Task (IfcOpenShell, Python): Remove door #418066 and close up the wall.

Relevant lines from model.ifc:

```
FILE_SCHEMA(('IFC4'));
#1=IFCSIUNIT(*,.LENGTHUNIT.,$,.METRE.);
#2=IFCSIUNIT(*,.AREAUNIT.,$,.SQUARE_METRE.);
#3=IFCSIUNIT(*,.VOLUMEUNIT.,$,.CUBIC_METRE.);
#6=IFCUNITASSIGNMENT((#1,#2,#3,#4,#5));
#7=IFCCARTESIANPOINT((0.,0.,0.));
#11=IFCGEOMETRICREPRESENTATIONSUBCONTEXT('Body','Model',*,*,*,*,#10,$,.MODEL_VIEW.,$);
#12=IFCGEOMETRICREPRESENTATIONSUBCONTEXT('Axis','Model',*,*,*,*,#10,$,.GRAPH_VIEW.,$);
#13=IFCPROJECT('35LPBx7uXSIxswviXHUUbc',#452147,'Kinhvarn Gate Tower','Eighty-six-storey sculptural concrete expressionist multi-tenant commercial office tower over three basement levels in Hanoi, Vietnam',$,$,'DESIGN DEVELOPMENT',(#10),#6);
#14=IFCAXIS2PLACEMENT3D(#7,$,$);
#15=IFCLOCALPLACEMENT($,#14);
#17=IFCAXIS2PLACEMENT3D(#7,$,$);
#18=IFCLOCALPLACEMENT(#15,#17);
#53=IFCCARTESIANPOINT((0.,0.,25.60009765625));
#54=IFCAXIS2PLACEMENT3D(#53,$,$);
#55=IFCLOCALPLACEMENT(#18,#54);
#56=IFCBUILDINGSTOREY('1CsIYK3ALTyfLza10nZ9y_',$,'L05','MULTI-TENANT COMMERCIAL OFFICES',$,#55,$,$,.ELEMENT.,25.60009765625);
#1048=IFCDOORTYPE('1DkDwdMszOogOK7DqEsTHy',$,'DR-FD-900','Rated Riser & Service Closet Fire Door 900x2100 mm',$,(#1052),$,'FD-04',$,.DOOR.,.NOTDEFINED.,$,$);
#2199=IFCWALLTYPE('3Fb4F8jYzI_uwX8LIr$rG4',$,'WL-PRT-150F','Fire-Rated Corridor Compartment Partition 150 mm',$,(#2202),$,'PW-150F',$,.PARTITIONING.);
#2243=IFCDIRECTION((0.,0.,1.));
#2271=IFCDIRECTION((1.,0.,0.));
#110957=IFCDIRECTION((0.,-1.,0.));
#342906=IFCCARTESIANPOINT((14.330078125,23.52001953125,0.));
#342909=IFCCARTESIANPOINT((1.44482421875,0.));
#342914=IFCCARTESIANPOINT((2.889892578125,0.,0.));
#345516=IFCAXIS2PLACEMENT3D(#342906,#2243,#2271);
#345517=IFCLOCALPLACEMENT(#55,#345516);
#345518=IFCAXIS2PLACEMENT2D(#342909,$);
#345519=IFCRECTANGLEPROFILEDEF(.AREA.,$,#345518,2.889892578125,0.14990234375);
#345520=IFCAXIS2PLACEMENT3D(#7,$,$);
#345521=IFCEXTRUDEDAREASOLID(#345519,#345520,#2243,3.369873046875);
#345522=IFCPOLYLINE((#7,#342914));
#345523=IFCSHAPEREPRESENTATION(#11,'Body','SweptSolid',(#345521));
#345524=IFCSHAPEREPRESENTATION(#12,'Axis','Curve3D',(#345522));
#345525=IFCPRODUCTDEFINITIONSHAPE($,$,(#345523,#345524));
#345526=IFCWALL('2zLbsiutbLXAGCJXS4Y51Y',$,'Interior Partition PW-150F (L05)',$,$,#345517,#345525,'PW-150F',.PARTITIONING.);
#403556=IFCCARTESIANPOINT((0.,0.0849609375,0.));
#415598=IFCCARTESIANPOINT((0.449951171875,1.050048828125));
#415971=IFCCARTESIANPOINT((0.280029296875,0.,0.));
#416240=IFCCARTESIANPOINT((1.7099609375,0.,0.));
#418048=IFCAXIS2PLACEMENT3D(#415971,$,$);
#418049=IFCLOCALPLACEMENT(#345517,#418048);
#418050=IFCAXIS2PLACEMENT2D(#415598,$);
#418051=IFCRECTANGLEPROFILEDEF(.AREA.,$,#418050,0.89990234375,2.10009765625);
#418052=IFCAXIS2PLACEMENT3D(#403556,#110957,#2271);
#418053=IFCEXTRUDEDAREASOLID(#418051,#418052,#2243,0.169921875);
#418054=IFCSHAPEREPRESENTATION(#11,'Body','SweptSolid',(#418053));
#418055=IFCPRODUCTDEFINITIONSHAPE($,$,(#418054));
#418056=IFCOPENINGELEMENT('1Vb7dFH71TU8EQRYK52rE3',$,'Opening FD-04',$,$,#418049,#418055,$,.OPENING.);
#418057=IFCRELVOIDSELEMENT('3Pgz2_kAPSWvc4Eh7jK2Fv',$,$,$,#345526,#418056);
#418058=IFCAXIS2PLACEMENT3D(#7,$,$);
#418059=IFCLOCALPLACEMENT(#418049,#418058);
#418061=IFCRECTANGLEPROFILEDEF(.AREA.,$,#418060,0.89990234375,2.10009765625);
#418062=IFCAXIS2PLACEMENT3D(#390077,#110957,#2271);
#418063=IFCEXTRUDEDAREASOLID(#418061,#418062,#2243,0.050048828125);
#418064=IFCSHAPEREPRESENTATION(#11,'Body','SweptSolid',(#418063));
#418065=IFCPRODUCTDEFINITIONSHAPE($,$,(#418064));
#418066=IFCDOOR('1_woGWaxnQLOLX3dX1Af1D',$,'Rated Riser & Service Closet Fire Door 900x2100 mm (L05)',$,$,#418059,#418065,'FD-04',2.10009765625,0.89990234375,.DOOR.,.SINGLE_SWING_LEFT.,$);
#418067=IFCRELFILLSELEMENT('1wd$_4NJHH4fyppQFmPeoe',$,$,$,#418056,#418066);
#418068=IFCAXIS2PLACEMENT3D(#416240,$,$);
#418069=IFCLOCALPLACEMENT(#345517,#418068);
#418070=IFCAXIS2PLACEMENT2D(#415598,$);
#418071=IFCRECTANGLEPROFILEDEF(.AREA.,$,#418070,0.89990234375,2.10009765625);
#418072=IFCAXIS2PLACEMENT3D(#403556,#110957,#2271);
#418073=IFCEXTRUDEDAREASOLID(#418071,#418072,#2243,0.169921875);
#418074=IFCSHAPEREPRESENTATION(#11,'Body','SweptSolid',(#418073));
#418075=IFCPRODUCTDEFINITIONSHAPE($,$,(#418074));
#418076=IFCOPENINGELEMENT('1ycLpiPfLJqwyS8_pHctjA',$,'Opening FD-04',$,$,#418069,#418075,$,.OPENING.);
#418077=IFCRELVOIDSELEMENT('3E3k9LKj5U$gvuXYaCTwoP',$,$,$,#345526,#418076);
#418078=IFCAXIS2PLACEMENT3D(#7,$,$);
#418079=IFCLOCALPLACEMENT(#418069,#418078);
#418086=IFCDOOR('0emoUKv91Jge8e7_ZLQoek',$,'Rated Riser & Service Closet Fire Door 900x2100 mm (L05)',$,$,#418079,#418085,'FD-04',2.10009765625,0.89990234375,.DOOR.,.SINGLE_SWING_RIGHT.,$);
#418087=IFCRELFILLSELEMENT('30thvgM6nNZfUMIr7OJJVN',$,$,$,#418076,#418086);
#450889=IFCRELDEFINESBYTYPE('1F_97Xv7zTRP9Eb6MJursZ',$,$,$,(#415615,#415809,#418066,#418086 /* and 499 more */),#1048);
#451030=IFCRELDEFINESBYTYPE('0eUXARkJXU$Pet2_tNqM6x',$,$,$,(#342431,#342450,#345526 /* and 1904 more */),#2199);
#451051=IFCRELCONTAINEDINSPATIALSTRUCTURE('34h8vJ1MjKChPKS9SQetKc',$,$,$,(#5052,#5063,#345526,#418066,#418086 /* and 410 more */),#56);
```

```python
import ifcopenshell
import ifcopenshell.api.feature
import ifcopenshell.api.root
import ifcopenshell.geom
import ifcopenshell.util.shape

model = ifcopenshell.open("model.ifc")
settings = ifcopenshell.geom.settings()


def volume(element):
    """Net volume in cubic metres, openings subtracted."""
    shape = ifcopenshell.geom.create_shape(settings, element)
    return ifcopenshell.util.shape.get_volume(shape.geometry)


door = model.by_guid("1_woGWaxnQLOLX3dX1Af1D")
opening = door.FillsVoids[0].RelatingOpeningElement
wall = opening.VoidsElements[0].RelatingBuildingElement
before = volume(wall)

ifcopenshell.api.root.remove_product(model, product=door)
ifcopenshell.api.feature.remove_feature(model, feature=opening)

after = volume(wall)

print(f"wall volume {before:.3f} -> {after:.3f} m3")

model.write("model_updated.ifc")
```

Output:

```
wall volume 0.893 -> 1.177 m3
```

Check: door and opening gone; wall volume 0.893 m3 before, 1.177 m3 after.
